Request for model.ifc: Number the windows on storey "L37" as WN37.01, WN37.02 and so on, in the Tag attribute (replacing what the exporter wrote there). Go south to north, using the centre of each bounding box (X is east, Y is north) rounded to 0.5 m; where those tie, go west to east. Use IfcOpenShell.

First a look at what the model holds.

```python
import ifcopenshell
import ifcopenshell.util.element
import ifcopenshell.util.placement

model = ifcopenshell.open("model.ifc")
print(model.schema)
storey = next(s for s in model.by_type("IfcBuildingStorey") if s.Name == "L37")
windows = [e for e in ifcopenshell.util.element.get_decomposition(storey) if e.is_a("IfcWindow")]
for e in sorted(windows, key=lambda e: e.id()):
    origin = ifcopenshell.util.placement.get_local_placement(e.ObjectPlacement)[:3, 3]
    print(e.id(), e.Tag, e.Name, origin.round(2) + 0.0, sep=" | ")
```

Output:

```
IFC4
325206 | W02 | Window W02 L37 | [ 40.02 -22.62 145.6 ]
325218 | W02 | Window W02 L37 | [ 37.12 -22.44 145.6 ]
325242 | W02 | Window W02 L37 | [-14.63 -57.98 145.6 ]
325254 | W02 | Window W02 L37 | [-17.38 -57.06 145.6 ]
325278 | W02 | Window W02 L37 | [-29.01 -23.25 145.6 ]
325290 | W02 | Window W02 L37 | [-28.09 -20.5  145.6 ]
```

```python
import ifcopenshell
import ifcopenshell.geom
import ifcopenshell.util.element
import ifcopenshell.util.shape

model = ifcopenshell.open("model.ifc")
settings = ifcopenshell.geom.settings()
settings.set("use-world-coords", True)


def centre(element):
    shape = ifcopenshell.geom.create_shape(settings, element)
    return ifcopenshell.util.shape.get_bbox_centroid(shape.geometry)


storey = next(s for s in model.by_type("IfcBuildingStorey") if s.Name == "L37")
windows = [e for e in ifcopenshell.util.element.get_decomposition(storey) if e.is_a("IfcWindow")]

# Insertion points can sit at a corner or the storey origin, so sort by the geometry (in metres).
centres = {e: centre(e) for e in windows}
windows.sort(key=lambda e: (round(centres[e][1] / 0.5), centres[e][0]))

for i, e in enumerate(windows, start=1):
    number = f"WN37.{i:02d}"
    e.Tag = number
    print(e.id(), number)

model.write("model_edited.ifc")
```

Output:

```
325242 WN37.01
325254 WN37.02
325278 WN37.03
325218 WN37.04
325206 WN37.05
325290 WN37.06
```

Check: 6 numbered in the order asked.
